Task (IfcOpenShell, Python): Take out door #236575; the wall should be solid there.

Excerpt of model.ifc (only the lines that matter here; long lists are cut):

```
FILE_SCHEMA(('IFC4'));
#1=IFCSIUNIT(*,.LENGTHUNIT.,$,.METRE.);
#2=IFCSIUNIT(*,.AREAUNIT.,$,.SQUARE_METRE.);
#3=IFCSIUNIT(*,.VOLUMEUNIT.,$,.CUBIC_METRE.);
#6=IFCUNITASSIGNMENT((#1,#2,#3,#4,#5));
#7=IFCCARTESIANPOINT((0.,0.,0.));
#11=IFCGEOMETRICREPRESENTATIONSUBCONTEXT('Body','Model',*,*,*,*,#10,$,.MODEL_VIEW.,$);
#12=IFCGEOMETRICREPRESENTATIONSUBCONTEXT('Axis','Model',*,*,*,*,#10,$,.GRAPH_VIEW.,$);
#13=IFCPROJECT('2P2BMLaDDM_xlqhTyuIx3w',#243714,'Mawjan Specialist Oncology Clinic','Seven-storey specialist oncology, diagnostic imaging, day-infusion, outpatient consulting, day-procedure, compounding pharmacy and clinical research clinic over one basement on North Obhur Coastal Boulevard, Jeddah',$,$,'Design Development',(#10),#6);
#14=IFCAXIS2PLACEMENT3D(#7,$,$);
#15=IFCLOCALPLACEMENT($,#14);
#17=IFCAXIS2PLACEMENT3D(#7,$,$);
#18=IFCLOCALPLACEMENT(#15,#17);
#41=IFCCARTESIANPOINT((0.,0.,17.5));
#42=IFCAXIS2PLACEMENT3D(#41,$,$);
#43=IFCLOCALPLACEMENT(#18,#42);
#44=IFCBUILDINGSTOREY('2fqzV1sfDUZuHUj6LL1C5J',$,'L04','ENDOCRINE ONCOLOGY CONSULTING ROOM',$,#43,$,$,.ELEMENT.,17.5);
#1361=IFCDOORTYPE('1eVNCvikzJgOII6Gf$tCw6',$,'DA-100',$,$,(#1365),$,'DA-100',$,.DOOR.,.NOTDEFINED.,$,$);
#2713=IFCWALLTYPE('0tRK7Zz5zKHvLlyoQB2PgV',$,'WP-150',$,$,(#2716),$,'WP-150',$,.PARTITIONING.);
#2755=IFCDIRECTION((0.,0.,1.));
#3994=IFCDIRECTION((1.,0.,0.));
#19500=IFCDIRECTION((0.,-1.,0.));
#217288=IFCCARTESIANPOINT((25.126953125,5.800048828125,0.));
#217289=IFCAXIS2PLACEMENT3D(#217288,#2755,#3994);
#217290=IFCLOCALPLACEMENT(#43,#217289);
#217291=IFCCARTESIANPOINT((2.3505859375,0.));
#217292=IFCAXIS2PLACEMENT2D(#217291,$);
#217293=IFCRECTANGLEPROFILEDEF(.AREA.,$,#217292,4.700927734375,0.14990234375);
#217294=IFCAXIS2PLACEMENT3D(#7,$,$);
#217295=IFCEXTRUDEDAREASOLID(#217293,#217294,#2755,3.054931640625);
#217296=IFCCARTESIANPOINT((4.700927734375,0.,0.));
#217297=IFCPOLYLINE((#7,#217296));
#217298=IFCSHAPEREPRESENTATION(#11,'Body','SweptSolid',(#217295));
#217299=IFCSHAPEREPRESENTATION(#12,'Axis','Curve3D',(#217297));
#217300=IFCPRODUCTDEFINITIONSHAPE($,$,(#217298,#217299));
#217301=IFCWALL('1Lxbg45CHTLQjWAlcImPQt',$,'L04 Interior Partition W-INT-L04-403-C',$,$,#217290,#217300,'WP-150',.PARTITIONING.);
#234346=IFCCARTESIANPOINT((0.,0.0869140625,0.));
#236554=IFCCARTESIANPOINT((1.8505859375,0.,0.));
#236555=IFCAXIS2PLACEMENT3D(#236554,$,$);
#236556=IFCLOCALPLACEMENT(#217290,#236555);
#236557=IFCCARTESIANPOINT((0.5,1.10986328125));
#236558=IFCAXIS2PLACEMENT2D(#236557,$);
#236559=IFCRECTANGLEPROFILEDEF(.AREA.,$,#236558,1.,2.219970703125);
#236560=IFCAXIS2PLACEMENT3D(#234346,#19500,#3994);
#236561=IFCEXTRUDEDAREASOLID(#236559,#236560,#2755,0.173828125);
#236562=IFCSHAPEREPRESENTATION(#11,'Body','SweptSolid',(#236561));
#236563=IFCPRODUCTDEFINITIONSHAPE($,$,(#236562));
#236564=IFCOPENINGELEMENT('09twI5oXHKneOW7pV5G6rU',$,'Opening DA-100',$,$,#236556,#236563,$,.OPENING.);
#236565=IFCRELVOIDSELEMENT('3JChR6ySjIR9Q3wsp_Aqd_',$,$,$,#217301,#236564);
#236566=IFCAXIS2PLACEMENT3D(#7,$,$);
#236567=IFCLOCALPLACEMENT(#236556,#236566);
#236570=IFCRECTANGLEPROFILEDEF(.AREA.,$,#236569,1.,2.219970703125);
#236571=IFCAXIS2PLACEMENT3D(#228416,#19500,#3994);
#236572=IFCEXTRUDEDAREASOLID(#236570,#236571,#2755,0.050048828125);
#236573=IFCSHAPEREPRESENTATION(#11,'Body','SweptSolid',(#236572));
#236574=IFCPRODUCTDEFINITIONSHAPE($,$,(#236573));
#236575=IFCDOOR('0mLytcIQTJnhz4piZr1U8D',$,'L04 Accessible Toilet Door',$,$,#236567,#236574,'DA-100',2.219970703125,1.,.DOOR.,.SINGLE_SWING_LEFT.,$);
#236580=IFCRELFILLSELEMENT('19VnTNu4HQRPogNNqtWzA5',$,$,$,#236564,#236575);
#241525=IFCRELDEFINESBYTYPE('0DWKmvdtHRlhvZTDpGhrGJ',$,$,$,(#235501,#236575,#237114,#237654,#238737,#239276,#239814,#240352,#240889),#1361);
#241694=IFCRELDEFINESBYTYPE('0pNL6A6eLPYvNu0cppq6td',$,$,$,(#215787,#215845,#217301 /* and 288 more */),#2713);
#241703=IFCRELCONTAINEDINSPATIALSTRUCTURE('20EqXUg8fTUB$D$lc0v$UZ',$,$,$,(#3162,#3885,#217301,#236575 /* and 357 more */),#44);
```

```python
import ifcopenshell
import ifcopenshell.api.feature
import ifcopenshell.api.root
import ifcopenshell.geom
import ifcopenshell.util.shape

model = ifcopenshell.open("model.ifc")
settings = ifcopenshell.geom.settings()


def volume(element):
    """Net volume in cubic metres, openings subtracted."""
    shape = ifcopenshell.geom.create_shape(settings, element)
    return ifcopenshell.util.shape.get_volume(shape.geometry)


door = model.by_guid("0mLytcIQTJnhz4piZr1U8D")
opening = door.FillsVoids[0].RelatingOpeningElement
wall = opening.VoidsElements[0].RelatingBuildingElement
before = volume(wall)

ifcopenshell.api.root.remove_product(model, product=door)
ifcopenshell.api.feature.remove_feature(model, feature=opening)

after = volume(wall)

print(f"wall volume {before:.3f} -> {after:.3f} m3")

model.write("model_edited.ifc")
```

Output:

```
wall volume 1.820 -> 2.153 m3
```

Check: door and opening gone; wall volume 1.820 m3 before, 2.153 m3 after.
